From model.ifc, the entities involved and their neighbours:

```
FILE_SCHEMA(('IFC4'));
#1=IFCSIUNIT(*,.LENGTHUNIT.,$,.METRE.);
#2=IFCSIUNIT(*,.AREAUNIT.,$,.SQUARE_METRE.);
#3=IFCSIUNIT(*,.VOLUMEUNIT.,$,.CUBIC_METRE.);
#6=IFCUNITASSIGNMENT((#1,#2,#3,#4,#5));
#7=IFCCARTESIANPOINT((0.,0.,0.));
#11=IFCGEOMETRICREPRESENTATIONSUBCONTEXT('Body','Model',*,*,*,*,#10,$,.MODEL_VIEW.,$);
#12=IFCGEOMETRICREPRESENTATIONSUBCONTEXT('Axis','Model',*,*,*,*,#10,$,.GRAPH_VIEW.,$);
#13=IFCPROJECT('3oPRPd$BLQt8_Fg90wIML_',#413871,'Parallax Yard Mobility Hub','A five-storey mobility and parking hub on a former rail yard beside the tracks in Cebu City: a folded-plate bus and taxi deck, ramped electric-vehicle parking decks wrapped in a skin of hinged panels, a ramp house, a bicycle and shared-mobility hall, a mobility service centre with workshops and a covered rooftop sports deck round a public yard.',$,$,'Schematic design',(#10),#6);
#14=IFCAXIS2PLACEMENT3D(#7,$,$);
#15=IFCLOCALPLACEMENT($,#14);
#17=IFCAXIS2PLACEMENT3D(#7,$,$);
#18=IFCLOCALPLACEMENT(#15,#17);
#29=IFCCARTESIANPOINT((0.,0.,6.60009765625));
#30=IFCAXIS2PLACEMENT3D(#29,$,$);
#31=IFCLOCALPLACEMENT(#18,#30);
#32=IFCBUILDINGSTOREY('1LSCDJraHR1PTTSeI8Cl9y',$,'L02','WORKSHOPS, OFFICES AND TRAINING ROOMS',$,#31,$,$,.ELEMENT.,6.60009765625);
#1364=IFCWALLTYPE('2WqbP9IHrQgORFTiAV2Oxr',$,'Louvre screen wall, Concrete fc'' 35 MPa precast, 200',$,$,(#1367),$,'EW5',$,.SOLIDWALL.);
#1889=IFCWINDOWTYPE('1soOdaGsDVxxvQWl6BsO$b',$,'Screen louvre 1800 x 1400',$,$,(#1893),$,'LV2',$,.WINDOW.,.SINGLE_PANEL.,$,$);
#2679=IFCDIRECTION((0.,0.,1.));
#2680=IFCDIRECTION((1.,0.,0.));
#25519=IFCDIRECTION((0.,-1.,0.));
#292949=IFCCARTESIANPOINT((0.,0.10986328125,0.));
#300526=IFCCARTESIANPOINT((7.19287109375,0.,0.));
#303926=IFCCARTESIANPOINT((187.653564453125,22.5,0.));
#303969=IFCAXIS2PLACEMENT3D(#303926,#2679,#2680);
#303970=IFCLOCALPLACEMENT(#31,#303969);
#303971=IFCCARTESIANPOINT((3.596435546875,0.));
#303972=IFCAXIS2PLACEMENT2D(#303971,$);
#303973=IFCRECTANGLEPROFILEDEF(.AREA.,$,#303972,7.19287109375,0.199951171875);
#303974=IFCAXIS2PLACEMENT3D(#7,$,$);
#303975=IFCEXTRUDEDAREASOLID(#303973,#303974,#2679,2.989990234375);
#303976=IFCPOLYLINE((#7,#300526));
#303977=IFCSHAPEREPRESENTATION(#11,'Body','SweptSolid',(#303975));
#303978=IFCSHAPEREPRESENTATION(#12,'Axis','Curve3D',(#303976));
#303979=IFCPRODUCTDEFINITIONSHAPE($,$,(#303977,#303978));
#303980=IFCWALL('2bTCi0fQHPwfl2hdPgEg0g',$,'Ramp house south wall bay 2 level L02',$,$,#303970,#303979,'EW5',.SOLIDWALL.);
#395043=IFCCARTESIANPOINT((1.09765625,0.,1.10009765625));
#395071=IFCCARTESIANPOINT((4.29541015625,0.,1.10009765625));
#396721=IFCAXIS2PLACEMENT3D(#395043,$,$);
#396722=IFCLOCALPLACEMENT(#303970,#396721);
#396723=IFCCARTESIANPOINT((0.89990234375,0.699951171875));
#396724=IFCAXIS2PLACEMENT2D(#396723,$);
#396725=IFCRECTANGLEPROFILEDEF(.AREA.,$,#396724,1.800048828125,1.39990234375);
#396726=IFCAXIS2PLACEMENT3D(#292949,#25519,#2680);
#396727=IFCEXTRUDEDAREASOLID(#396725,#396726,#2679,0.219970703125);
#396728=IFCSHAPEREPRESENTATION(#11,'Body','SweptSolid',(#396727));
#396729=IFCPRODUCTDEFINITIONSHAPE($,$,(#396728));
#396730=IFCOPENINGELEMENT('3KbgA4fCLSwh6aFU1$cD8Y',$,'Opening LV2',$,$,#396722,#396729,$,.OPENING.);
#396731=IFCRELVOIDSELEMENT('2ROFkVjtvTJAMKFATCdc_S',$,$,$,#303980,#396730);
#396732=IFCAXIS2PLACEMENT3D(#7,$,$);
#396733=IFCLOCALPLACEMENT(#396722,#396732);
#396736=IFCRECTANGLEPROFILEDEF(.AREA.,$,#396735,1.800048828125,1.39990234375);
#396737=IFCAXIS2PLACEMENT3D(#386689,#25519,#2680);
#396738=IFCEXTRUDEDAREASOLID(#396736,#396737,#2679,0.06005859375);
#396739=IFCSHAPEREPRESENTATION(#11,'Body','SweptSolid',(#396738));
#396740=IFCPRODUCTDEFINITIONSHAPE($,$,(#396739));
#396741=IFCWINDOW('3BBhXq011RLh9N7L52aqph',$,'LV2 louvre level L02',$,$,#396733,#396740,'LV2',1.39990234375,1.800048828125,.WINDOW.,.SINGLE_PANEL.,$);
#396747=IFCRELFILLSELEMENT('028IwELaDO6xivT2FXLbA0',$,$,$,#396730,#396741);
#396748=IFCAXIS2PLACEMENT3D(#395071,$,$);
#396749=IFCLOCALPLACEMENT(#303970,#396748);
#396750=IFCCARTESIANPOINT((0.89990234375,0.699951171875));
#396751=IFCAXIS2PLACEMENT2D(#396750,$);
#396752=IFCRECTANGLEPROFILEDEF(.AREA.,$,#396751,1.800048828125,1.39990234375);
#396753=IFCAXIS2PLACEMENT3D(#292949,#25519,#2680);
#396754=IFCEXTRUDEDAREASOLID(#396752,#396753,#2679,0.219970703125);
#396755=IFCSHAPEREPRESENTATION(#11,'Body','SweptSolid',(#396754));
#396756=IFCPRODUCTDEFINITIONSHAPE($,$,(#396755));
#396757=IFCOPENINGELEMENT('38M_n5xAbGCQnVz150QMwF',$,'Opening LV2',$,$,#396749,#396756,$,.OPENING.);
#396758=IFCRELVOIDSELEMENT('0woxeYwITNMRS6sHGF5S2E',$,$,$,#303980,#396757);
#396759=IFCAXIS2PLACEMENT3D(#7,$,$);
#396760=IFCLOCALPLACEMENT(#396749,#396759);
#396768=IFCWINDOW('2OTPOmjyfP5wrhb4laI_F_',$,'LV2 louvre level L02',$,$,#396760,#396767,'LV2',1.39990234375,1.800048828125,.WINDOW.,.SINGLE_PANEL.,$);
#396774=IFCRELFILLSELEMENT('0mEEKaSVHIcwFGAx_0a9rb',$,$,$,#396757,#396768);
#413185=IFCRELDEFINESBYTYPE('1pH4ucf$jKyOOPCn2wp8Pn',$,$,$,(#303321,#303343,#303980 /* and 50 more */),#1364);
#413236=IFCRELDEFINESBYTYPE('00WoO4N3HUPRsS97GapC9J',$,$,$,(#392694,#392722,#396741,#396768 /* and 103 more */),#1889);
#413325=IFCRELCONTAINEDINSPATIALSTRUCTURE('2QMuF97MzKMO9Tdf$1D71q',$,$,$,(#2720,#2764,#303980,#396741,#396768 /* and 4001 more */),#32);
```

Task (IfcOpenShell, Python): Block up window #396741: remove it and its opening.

```python
import ifcopenshell
import ifcopenshell.api.feature
import ifcopenshell.api.root
import ifcopenshell.geom
import ifcopenshell.util.shape

model = ifcopenshell.open("model.ifc")
settings = ifcopenshell.geom.settings()


def volume(element):
    """Net volume in cubic metres, openings subtracted."""
    shape = ifcopenshell.geom.create_shape(settings, element)
    return ifcopenshell.util.shape.get_volume(shape.geometry)


window = model.by_guid("3BBhXq011RLh9N7L52aqph")
opening = window.FillsVoids[0].RelatingOpeningElement
wall = opening.VoidsElements[0].RelatingBuildingElement
before = volume(wall)

ifcopenshell.api.root.remove_product(model, product=window)
ifcopenshell.api.feature.remove_feature(model, feature=opening)

after = volume(wall)

print(f"wall volume {before:.3f} -> {after:.3f} m3")

model.write("model-out.ifc")
```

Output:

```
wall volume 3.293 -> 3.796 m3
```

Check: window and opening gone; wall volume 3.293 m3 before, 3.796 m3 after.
